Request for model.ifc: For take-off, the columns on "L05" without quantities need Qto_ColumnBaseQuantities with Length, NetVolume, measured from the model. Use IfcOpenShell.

First a look at what the model holds.

```python
import ifcopenshell
import ifcopenshell.util.element
import ifcopenshell.util.unit

model = ifcopenshell.open("model.ifc")
print(model.schema)
for unit_type in ("LENGTHUNIT", "AREAUNIT", "VOLUMEUNIT"):
    print(unit_type, ifcopenshell.util.unit.calculate_unit_scale(model, unit_type))
storey = next(s for s in model.by_type("IfcBuildingStorey") if s.Name == "L05")
columns = [e for e in ifcopenshell.util.element.get_decomposition(storey) if e.is_a("IfcColumn")]
for e in sorted(columns, key=lambda e: e.id()):
    print(e.id(), e.is_a(), e.Name, list(ifcopenshell.util.element.get_psets(e, qtos_only=True)), sep=" | ")
```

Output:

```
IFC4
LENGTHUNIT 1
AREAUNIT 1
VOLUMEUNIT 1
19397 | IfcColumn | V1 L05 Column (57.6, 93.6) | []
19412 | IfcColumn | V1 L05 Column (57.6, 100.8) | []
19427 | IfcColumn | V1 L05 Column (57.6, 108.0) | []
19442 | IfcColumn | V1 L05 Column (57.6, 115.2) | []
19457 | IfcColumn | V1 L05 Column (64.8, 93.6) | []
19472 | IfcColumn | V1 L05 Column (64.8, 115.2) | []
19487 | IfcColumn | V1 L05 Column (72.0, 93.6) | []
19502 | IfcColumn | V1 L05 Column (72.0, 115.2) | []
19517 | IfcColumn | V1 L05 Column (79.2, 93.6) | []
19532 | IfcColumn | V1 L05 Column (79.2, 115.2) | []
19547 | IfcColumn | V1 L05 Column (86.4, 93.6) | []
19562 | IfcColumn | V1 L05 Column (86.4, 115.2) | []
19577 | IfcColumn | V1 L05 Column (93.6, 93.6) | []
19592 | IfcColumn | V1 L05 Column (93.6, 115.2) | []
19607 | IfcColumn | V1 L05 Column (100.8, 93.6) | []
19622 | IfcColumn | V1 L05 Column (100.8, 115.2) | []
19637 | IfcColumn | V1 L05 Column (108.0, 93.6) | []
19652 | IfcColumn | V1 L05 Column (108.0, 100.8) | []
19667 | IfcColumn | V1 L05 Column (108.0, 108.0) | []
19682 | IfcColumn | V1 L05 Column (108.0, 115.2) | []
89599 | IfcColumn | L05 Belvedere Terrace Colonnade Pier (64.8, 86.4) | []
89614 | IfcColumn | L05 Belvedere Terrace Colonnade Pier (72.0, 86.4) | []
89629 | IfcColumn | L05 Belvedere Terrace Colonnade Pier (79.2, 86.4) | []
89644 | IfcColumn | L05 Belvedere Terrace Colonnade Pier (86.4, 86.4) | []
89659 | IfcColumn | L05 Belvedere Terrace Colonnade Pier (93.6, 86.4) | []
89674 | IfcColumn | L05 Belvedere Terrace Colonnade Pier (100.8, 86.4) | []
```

```python
import ifcopenshell
import ifcopenshell.api.pset
import ifcopenshell.geom
import ifcopenshell.util.element
import ifcopenshell.util.shape
import ifcopenshell.util.unit

model = ifcopenshell.open("model.ifc")
unit_scale = ifcopenshell.util.unit.calculate_unit_scale(model)
volume_scale = ifcopenshell.util.unit.calculate_unit_scale(model, "VOLUMEUNIT")
settings = ifcopenshell.geom.settings()

storey = next(s for s in model.by_type("IfcBuildingStorey") if s.Name == "L05")
columns = [e for e in ifcopenshell.util.element.get_decomposition(storey) if e.is_a("IfcColumn")]

for e in sorted(columns, key=lambda e: e.id()):
    if ifcopenshell.util.element.get_psets(e, qtos_only=True, should_inherit=False):
        continue
    # Geometry comes back in metres, in the element's own axes.
    shape = ifcopenshell.geom.create_shape(settings, e)
    values = {
        "Length": ifcopenshell.util.shape.get_z(shape.geometry) / unit_scale,
        "NetVolume": ifcopenshell.util.shape.get_volume(shape.geometry) / volume_scale,
    }
    qto = ifcopenshell.api.pset.add_qto(model, product=e, name="Qto_ColumnBaseQuantities")
    ifcopenshell.api.pset.edit_qto(model, qto=qto, properties=values)
    print(e.id(), {k: round(v, 3) for k, v in values.items()})

model.write("model_edited.ifc")
```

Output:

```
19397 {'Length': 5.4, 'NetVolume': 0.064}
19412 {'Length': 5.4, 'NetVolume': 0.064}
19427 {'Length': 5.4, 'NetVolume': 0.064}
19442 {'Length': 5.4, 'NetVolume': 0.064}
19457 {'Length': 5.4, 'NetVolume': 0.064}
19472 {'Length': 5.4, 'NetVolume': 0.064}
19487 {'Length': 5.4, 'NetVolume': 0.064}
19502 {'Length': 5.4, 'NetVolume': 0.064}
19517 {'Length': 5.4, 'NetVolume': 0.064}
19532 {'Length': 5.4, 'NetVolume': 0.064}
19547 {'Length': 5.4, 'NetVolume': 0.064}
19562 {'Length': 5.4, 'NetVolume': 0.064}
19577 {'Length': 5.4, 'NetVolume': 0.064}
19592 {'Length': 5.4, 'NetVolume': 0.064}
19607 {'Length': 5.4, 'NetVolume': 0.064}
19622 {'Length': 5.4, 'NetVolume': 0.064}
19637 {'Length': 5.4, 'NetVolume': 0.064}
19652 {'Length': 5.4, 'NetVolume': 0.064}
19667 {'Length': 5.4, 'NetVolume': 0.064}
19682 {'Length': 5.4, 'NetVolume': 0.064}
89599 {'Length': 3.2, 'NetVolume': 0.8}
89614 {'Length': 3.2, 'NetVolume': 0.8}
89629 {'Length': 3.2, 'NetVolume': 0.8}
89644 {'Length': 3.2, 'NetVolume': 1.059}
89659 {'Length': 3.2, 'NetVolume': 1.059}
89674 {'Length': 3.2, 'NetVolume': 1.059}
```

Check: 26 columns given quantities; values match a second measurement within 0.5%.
